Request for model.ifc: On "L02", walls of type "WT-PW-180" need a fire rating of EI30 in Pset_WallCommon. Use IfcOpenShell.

First a look at what the model holds.

```python
import ifcopenshell
import ifcopenshell.util.element

model = ifcopenshell.open("model.ifc")
print(model.schema)
storey = next(s for s in model.by_type("IfcBuildingStorey") if s.Name == "L02")
walls = [e for e in ifcopenshell.util.element.get_decomposition(storey) if e.is_a("IfcWall")]
seen = {}
for e in walls:
    element_type = ifcopenshell.util.element.get_type(e)
    key = (element_type.Name if element_type != e and element_type else None, ifcopenshell.util.element.get_pset(e, "Pset_WallCommon", "FireRating"))
    seen[key] = seen.get(key, 0) + 1
for (name, value), count in sorted(seen.items(), key=str):
    print(count, "x", name, "|", value)
```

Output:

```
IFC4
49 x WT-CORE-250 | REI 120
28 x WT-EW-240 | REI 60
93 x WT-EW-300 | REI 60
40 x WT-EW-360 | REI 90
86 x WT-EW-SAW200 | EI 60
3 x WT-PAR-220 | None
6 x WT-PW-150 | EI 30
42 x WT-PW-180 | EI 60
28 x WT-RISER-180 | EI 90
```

```python
import ifcopenshell
import ifcopenshell.api.pset
import ifcopenshell.util.element

model = ifcopenshell.open("model.ifc")

storey = next(s for s in model.by_type("IfcBuildingStorey") if s.Name == "L02")
walls = [e for e in ifcopenshell.util.element.get_decomposition(storey) if e.is_a("IfcWall")]

count = 0
for e in walls:
    element_type = ifcopenshell.util.element.get_type(e)
    if element_type in (None, e) or element_type.Name != "WT-PW-180":
        continue
    # add_pset returns the element's existing set when there is one.
    pset = ifcopenshell.api.pset.add_pset(model, product=e, name="Pset_WallCommon")
    ifcopenshell.api.pset.edit_pset(model, pset=pset, properties={"FireRating": "EI30"})
    count += 1

print(count, "walls updated")

model.write("model-out.ifc")
```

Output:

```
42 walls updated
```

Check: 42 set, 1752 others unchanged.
